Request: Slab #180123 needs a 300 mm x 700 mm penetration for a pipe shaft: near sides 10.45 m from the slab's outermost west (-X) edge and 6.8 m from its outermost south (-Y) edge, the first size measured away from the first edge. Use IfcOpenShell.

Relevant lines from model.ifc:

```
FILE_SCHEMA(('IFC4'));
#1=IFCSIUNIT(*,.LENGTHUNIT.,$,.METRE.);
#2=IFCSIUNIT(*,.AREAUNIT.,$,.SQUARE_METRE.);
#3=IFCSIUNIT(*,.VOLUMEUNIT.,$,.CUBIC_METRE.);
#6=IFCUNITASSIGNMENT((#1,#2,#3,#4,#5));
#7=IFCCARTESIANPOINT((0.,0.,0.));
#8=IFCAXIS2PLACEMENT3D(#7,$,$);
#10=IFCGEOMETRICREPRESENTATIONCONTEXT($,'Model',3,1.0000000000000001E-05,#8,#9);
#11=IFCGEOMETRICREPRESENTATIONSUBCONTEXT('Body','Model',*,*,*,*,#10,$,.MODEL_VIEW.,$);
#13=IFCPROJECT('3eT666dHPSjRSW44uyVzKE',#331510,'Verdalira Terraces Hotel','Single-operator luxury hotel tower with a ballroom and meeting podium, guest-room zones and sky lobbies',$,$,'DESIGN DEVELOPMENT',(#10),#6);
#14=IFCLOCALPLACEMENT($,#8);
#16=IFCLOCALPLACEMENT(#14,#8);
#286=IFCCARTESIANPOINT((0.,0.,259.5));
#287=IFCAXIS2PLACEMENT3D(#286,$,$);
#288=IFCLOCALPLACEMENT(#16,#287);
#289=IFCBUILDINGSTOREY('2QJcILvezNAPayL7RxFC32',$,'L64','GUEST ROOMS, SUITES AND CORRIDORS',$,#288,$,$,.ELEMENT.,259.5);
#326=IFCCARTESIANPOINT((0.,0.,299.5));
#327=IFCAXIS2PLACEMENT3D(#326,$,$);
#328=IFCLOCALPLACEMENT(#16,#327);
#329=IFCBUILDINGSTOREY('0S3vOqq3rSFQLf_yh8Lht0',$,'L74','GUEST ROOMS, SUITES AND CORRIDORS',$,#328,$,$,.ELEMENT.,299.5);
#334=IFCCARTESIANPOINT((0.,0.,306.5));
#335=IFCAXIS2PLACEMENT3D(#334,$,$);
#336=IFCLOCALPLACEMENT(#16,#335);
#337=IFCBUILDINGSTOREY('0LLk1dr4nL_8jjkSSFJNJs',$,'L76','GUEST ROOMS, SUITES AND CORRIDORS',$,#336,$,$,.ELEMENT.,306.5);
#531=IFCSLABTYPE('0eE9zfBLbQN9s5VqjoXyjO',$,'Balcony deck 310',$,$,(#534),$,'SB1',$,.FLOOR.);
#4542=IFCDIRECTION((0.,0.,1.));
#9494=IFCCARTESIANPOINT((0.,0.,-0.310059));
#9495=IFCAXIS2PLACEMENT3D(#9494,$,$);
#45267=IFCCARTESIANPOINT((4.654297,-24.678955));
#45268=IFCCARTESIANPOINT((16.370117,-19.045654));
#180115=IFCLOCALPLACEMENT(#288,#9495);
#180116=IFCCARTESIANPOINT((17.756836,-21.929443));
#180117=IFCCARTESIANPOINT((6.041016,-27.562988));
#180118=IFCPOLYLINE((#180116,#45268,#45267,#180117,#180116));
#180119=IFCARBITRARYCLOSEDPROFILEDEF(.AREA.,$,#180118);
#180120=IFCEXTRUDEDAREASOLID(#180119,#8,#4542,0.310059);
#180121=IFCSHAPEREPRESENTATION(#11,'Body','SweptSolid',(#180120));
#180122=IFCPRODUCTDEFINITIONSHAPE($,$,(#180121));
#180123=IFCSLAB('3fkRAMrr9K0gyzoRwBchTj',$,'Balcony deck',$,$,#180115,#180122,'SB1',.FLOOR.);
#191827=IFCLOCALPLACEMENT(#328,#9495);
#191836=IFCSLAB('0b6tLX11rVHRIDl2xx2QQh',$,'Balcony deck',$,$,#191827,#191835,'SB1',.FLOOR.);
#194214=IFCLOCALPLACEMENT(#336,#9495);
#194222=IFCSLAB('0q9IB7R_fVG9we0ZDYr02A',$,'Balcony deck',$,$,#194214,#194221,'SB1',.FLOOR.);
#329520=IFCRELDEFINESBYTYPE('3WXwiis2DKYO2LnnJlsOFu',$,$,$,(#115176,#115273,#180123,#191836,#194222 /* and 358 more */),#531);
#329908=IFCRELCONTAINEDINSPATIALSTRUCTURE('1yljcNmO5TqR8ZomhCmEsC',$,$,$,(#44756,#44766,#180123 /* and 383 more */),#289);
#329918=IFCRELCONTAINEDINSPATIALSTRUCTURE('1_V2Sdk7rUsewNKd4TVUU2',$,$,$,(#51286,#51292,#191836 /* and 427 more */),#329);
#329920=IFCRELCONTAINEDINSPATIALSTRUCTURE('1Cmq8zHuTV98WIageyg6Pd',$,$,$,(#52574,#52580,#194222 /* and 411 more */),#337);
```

```python
import numpy as np
import ifcopenshell
import ifcopenshell.api.feature
import ifcopenshell.api.geometry
import ifcopenshell.api.root
import ifcopenshell.geom
import ifcopenshell.util.placement
import ifcopenshell.util.representation
import ifcopenshell.util.shape
import ifcopenshell.util.unit

model = ifcopenshell.open("model.ifc")
unit_scale = ifcopenshell.util.unit.calculate_unit_scale(model)
settings = ifcopenshell.geom.settings()


def volume(element):
    """Net volume in cubic metres, openings subtracted."""
    shape = ifcopenshell.geom.create_shape(settings, element)
    return ifcopenshell.util.shape.get_volume(shape.geometry)


slab = model.by_guid("3fkRAMrr9K0gyzoRwBchTj")
before = volume(slab)

# Extent in the slab's own axes, in metres. The edges named are its -X and -Y sides.
slab_shape = ifcopenshell.geom.create_shape(settings, slab)
vertices = ifcopenshell.util.shape.get_vertices(slab_shape.geometry)
x_min, y_min, bottom = vertices.min(axis=0)
top = vertices[:, 2].max()

opening = ifcopenshell.api.root.create_entity(model, ifc_class="IfcOpeningElement", name="Pipe shaft opening", predefined_type="OPENING")
context = ifcopenshell.util.representation.get_context(model, "Model", "Body", "MODEL_VIEW")
width, depth = 0.3, 0.7
outline = [(0.0, 0.0), (width, 0.0), (width, depth), (0.0, depth), (0.0, 0.0)]
# Overshoot both faces by 50 mm so the cut is clean.
shape = ifcopenshell.api.geometry.add_slab_representation(
    model, context=context, depth=top - bottom + 0.1, polyline=outline
)
ifcopenshell.api.geometry.assign_representation(model, product=opening, representation=shape)

matrix = ifcopenshell.util.placement.get_local_placement(slab.ObjectPlacement)
matrix[:, 3] = matrix @ np.append(np.array([x_min + 10.45, y_min + 6.8, bottom - 0.05]) / unit_scale, 1.0)
ifcopenshell.api.geometry.edit_object_placement(model, product=opening, matrix=matrix, is_si=False)
ifcopenshell.api.feature.add_feature(model, feature=opening, element=slab)

after = volume(slab)

print(f"slab volume {before:.3f} -> {after:.3f} m3")

model.write("model_rev.ifc")
```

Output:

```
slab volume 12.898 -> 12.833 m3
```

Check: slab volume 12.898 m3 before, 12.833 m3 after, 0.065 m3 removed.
